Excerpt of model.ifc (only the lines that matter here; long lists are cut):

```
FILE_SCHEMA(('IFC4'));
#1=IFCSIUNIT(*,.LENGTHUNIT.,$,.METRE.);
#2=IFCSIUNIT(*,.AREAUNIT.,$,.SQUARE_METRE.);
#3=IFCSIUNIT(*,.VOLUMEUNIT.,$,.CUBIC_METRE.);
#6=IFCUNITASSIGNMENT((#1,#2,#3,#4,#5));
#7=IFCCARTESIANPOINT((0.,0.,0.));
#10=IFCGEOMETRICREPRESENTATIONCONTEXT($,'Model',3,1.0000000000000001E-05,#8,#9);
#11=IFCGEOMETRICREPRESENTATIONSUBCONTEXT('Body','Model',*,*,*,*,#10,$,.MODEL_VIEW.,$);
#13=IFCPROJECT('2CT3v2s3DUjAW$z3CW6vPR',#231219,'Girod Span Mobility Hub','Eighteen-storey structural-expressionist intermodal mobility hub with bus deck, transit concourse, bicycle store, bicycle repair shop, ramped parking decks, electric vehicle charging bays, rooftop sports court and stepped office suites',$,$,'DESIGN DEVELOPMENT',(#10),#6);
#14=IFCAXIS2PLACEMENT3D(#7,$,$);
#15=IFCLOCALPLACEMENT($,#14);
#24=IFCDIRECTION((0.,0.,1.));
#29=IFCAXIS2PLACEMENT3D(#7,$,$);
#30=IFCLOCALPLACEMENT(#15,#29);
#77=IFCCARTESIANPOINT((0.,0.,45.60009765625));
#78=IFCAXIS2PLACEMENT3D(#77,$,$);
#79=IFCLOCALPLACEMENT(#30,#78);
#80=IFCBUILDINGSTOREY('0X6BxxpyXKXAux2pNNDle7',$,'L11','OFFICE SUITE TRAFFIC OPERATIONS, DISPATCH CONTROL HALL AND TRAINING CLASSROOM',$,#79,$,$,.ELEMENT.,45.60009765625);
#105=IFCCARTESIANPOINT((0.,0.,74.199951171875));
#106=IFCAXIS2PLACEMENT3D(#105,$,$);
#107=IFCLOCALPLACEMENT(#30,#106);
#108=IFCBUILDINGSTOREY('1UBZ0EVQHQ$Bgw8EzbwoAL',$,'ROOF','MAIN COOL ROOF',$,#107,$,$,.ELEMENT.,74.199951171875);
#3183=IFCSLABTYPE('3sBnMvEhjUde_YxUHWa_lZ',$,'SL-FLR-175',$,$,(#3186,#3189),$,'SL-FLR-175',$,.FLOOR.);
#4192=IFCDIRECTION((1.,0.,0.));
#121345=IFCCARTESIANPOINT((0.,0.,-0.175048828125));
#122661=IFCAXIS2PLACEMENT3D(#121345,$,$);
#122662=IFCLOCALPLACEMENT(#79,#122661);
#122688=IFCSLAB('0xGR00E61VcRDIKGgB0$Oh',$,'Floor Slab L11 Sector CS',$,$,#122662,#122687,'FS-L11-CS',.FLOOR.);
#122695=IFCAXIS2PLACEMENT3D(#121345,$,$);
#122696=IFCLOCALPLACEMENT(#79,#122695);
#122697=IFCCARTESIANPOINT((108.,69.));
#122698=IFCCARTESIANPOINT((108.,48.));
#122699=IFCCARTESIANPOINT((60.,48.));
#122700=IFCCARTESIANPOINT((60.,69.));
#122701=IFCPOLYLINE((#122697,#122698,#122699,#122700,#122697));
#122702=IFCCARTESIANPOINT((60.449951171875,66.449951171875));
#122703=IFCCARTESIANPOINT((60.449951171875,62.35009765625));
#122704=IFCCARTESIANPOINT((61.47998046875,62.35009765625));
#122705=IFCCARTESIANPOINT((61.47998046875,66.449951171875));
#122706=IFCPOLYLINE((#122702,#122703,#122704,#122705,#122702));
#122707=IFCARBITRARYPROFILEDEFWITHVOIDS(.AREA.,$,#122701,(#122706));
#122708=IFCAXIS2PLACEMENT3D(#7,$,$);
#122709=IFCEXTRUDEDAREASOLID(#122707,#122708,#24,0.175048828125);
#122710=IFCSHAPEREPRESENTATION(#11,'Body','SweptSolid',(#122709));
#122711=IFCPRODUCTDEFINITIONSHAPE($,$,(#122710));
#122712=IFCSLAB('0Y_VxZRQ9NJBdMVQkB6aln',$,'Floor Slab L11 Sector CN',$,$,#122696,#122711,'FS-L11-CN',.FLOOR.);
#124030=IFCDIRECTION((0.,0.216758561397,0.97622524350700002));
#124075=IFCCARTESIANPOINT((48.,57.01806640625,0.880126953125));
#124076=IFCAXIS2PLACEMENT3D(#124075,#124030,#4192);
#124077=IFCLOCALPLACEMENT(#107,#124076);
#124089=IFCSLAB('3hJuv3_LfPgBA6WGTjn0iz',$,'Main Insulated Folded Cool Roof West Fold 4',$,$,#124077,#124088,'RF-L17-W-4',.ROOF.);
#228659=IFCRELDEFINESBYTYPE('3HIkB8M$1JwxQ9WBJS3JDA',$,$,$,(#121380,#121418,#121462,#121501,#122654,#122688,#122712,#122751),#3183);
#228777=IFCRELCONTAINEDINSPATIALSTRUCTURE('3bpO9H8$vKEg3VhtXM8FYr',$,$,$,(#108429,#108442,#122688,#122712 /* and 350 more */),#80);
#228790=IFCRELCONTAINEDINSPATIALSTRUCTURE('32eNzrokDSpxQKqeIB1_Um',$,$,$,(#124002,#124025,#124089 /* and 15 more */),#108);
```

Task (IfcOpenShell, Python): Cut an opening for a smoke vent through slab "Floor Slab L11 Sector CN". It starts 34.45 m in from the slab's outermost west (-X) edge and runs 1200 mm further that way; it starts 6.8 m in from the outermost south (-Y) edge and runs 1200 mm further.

```python
import numpy as np
import ifcopenshell
import ifcopenshell.api.feature
import ifcopenshell.api.geometry
import ifcopenshell.api.root
import ifcopenshell.geom
import ifcopenshell.util.placement
import ifcopenshell.util.representation
import ifcopenshell.util.shape
import ifcopenshell.util.unit

model = ifcopenshell.open("model.ifc")
unit_scale = ifcopenshell.util.unit.calculate_unit_scale(model)
settings = ifcopenshell.geom.settings()


def volume(element):
    """Net volume in cubic metres, openings subtracted."""
    shape = ifcopenshell.geom.create_shape(settings, element)
    return ifcopenshell.util.shape.get_volume(shape.geometry)


slab = model.by_id(122712)
before = volume(slab)

# Extent in the slab's own axes, in metres. The edges named are its -X and -Y sides.
slab_shape = ifcopenshell.geom.create_shape(settings, slab)
vertices = ifcopenshell.util.shape.get_vertices(slab_shape.geometry)
x_min, y_min, bottom = vertices.min(axis=0)
top = vertices[:, 2].max()

opening = ifcopenshell.api.root.create_entity(model, ifc_class="IfcOpeningElement", name="Smoke vent opening", predefined_type="OPENING")
context = ifcopenshell.util.representation.get_context(model, "Model", "Body", "MODEL_VIEW")
width, depth = 1.2, 1.2
outline = [(0.0, 0.0), (width, 0.0), (width, depth), (0.0, depth), (0.0, 0.0)]
# Overshoot both faces by 50 mm so the cut is clean.
shape = ifcopenshell.api.geometry.add_slab_representation(
    model, context=context, depth=top - bottom + 0.1, polyline=outline
)
ifcopenshell.api.geometry.assign_representation(model, product=opening, representation=shape)

matrix = ifcopenshell.util.placement.get_local_placement(slab.ObjectPlacement)
matrix[:, 3] = matrix @ np.append(np.array([x_min + 34.45, y_min + 6.8, bottom - 0.05]) / unit_scale, 1.0)
ifcopenshell.api.geometry.edit_object_placement(model, product=opening, matrix=matrix, is_si=False)
ifcopenshell.api.feature.add_feature(model, feature=opening, element=slab)

after = volume(slab)

print(f"slab volume {before:.3f} -> {after:.3f} m3")

model.write("model_v2.ifc")
```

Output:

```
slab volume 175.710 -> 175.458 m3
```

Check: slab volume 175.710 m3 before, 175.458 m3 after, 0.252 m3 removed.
